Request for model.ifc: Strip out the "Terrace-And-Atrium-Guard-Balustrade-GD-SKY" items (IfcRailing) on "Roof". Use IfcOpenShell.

First a look at what the model holds.

```python
import ifcopenshell
import ifcopenshell.util.element

model = ifcopenshell.open("model.ifc")
print(model.schema)
storey = next(s for s in model.by_type("IfcBuildingStorey") if s.Name == "Roof")
railings = [e for e in ifcopenshell.util.element.get_decomposition(storey) if e.is_a("IfcRailing")]
seen = {}
for e in railings:
    element_type = ifcopenshell.util.element.get_type(e)
    name = element_type.Name if element_type not in (None, e) else None
    seen[name] = seen.get(name, 0) + 1
for name, count in sorted(seen.items(), key=str):
    print(count, "x", name)
```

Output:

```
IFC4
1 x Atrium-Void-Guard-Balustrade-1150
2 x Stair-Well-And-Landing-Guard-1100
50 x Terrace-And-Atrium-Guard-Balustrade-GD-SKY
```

```python
import ifcopenshell
import ifcopenshell.api.root
import ifcopenshell.util.element

model = ifcopenshell.open("model.ifc")

storey = next(s for s in model.by_type("IfcBuildingStorey") if s.Name == "Roof")
railings = [e for e in ifcopenshell.util.element.get_decomposition(storey) if e.is_a("IfcRailing")]
targets = [e for e in railings if (t := ifcopenshell.util.element.get_type(e)) not in (None, e) and t.Name == "Terrace-And-Atrium-Guard-Balustrade-GD-SKY"]

for e in targets:
    ifcopenshell.api.root.remove_product(model, product=e)
print(len(targets), "removed")

model.write("model-out.ifc")
```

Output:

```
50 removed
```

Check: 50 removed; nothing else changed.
